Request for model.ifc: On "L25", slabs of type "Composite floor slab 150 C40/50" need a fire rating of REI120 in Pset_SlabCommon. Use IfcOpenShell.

First a look at what the model holds.

```python
import ifcopenshell
import ifcopenshell.util.element

model = ifcopenshell.open("model.ifc")
print(model.schema)
storey = next(s for s in model.by_type("IfcBuildingStorey") if s.Name == "L25")
slabs = [e for e in ifcopenshell.util.element.get_decomposition(storey) if e.is_a("IfcSlab")]
seen = {}
for e in slabs:
    element_type = ifcopenshell.util.element.get_type(e)
    key = (element_type.Name if element_type != e and element_type else None, ifcopenshell.util.element.get_pset(e, "Pset_SlabCommon", "FireRating"))
    seen[key] = seen.get(key, 0) + 1
for (name, value), count in sorted(seen.items(), key=str):
    print(count, "x", name, "|", value)
```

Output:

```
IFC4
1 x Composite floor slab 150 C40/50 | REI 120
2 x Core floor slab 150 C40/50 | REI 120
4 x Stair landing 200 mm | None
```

```python
import ifcopenshell
import ifcopenshell.api.pset
import ifcopenshell.util.element

model = ifcopenshell.open("model.ifc")

storey = next(s for s in model.by_type("IfcBuildingStorey") if s.Name == "L25")
slabs = [e for e in ifcopenshell.util.element.get_decomposition(storey) if e.is_a("IfcSlab")]

count = 0
for e in slabs:
    element_type = ifcopenshell.util.element.get_type(e)
    if element_type in (None, e) or element_type.Name != "Composite floor slab 150 C40/50":
        continue
    found = ifcopenshell.util.element.get_pset(e, "Pset_SlabCommon", should_inherit=False)
    if found:
        pset = model.by_id(found["id"])
        if len(ifcopenshell.util.element.get_elements_by_pset(pset)) > 1:
            pset = ifcopenshell.api.pset.unshare_pset(model, products=[e], pset=pset)[0]
    else:
        pset = ifcopenshell.api.pset.add_pset(model, product=e, name="Pset_SlabCommon")
    ifcopenshell.api.pset.edit_pset(model, pset=pset, properties={"FireRating": "REI120"})
    count += 1

print(count, "slabs updated")

model.write("model_v2.ifc")
```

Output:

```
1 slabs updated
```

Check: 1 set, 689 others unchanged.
